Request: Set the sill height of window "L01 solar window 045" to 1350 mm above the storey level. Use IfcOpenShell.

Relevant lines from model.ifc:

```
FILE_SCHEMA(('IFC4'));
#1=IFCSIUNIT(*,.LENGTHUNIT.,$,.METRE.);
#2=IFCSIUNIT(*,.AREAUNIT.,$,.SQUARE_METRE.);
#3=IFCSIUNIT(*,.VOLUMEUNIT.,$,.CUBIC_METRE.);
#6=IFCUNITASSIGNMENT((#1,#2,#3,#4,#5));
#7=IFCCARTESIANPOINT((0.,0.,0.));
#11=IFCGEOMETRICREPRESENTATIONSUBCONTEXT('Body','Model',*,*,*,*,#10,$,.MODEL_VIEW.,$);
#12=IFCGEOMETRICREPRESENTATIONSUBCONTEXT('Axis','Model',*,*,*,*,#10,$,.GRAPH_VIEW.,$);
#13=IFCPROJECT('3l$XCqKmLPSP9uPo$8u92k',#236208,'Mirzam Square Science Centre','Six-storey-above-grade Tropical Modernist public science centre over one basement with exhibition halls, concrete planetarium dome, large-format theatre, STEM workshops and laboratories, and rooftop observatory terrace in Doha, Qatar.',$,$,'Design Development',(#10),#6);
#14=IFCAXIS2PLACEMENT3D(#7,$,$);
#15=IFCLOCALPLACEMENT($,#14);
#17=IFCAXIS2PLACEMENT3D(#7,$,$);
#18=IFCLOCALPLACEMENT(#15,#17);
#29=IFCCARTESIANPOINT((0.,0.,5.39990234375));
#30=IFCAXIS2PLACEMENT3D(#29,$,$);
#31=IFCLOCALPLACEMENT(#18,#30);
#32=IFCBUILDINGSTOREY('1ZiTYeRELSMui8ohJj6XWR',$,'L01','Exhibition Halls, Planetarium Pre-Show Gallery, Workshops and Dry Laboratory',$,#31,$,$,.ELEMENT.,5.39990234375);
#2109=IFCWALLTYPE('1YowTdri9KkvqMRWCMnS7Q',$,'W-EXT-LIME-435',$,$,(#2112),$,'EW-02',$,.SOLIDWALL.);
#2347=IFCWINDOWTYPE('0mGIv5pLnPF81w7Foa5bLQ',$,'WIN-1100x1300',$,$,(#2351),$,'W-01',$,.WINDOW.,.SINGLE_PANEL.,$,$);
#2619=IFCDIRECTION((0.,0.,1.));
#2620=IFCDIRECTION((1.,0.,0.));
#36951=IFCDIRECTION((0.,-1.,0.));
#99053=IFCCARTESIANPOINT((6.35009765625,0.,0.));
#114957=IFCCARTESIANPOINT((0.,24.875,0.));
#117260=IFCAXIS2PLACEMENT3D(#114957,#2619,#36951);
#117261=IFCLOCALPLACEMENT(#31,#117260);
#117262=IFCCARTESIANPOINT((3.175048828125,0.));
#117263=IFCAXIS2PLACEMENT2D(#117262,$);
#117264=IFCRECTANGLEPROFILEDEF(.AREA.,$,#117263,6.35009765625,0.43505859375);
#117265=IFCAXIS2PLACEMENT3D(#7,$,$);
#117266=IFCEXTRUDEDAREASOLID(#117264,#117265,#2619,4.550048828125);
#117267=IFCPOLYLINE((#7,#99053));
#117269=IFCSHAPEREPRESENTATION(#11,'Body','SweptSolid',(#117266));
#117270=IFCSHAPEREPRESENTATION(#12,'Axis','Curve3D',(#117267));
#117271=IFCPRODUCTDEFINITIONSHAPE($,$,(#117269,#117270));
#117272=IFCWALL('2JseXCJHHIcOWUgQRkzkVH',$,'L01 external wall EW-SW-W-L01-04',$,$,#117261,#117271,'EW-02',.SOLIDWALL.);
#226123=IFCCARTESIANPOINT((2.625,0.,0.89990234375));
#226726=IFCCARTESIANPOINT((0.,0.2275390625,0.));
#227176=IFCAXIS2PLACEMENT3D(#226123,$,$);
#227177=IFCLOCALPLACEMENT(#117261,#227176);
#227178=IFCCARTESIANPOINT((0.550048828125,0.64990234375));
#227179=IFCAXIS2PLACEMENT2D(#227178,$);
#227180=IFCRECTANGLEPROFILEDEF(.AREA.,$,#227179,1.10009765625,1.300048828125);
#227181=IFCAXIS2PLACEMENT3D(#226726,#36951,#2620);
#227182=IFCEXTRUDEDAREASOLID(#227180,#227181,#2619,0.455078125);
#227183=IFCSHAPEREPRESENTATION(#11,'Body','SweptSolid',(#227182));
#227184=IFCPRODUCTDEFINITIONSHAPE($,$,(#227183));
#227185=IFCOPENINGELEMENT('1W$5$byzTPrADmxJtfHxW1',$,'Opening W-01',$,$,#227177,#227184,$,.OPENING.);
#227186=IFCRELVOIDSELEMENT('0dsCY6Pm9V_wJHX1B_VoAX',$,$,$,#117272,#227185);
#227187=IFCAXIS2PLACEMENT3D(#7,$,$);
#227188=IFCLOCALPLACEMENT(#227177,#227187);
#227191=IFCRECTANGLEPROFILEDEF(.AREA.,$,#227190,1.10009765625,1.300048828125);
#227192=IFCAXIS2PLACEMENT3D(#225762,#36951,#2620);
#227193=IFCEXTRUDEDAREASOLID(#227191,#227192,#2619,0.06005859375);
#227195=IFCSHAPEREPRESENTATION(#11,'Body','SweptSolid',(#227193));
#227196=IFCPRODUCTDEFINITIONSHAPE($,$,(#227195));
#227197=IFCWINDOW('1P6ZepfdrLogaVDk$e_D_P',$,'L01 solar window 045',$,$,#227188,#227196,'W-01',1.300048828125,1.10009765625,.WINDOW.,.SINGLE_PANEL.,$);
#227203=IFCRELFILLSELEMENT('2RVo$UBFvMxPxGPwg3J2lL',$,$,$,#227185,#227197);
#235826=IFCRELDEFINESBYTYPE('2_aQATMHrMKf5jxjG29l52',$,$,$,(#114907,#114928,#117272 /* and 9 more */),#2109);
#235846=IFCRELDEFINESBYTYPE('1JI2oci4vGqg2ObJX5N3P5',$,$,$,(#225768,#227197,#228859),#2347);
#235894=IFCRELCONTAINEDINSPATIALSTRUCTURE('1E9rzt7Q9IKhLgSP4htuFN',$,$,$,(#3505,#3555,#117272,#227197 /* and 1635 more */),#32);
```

```python
import numpy as np
import ifcopenshell
import ifcopenshell.api.geometry
import ifcopenshell.geom
import ifcopenshell.util.element
import ifcopenshell.util.placement
import ifcopenshell.util.shape
import ifcopenshell.util.unit

model = ifcopenshell.open("model.ifc")
unit_scale = ifcopenshell.util.unit.calculate_unit_scale(model)

window = model.by_guid("1P6ZepfdrLogaVDk$e_D_P")
opening = window.FillsVoids[0].RelatingOpeningElement
storey = ifcopenshell.util.element.get_container(window, ifc_class="IfcBuildingStorey")
level = ifcopenshell.util.placement.get_local_placement(storey.ObjectPlacement)[2, 3]

# The opening's origin need not be at the sill, so measure its lowest point.
shape = ifcopenshell.geom.create_shape(ifcopenshell.geom.settings(), opening)
bottom = ifcopenshell.util.shape.get_shape_bottom_elevation(shape, shape.geometry) / unit_scale
dz = level + 1.35 - bottom

shift = np.array([0.0, 0.0, dz])
# The window is placed relative to its opening, so it follows when the opening moves.
matrix = ifcopenshell.util.placement.get_local_placement(opening.ObjectPlacement)
matrix[:3, 3] += shift
ifcopenshell.api.geometry.edit_object_placement(
    model, product=opening, matrix=matrix, is_si=False, should_transform_children=True
)

print(f"moved by {dz * unit_scale:+.3f} m")

model.write("model_rev.ifc")
```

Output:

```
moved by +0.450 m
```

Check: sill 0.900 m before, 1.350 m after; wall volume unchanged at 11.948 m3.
